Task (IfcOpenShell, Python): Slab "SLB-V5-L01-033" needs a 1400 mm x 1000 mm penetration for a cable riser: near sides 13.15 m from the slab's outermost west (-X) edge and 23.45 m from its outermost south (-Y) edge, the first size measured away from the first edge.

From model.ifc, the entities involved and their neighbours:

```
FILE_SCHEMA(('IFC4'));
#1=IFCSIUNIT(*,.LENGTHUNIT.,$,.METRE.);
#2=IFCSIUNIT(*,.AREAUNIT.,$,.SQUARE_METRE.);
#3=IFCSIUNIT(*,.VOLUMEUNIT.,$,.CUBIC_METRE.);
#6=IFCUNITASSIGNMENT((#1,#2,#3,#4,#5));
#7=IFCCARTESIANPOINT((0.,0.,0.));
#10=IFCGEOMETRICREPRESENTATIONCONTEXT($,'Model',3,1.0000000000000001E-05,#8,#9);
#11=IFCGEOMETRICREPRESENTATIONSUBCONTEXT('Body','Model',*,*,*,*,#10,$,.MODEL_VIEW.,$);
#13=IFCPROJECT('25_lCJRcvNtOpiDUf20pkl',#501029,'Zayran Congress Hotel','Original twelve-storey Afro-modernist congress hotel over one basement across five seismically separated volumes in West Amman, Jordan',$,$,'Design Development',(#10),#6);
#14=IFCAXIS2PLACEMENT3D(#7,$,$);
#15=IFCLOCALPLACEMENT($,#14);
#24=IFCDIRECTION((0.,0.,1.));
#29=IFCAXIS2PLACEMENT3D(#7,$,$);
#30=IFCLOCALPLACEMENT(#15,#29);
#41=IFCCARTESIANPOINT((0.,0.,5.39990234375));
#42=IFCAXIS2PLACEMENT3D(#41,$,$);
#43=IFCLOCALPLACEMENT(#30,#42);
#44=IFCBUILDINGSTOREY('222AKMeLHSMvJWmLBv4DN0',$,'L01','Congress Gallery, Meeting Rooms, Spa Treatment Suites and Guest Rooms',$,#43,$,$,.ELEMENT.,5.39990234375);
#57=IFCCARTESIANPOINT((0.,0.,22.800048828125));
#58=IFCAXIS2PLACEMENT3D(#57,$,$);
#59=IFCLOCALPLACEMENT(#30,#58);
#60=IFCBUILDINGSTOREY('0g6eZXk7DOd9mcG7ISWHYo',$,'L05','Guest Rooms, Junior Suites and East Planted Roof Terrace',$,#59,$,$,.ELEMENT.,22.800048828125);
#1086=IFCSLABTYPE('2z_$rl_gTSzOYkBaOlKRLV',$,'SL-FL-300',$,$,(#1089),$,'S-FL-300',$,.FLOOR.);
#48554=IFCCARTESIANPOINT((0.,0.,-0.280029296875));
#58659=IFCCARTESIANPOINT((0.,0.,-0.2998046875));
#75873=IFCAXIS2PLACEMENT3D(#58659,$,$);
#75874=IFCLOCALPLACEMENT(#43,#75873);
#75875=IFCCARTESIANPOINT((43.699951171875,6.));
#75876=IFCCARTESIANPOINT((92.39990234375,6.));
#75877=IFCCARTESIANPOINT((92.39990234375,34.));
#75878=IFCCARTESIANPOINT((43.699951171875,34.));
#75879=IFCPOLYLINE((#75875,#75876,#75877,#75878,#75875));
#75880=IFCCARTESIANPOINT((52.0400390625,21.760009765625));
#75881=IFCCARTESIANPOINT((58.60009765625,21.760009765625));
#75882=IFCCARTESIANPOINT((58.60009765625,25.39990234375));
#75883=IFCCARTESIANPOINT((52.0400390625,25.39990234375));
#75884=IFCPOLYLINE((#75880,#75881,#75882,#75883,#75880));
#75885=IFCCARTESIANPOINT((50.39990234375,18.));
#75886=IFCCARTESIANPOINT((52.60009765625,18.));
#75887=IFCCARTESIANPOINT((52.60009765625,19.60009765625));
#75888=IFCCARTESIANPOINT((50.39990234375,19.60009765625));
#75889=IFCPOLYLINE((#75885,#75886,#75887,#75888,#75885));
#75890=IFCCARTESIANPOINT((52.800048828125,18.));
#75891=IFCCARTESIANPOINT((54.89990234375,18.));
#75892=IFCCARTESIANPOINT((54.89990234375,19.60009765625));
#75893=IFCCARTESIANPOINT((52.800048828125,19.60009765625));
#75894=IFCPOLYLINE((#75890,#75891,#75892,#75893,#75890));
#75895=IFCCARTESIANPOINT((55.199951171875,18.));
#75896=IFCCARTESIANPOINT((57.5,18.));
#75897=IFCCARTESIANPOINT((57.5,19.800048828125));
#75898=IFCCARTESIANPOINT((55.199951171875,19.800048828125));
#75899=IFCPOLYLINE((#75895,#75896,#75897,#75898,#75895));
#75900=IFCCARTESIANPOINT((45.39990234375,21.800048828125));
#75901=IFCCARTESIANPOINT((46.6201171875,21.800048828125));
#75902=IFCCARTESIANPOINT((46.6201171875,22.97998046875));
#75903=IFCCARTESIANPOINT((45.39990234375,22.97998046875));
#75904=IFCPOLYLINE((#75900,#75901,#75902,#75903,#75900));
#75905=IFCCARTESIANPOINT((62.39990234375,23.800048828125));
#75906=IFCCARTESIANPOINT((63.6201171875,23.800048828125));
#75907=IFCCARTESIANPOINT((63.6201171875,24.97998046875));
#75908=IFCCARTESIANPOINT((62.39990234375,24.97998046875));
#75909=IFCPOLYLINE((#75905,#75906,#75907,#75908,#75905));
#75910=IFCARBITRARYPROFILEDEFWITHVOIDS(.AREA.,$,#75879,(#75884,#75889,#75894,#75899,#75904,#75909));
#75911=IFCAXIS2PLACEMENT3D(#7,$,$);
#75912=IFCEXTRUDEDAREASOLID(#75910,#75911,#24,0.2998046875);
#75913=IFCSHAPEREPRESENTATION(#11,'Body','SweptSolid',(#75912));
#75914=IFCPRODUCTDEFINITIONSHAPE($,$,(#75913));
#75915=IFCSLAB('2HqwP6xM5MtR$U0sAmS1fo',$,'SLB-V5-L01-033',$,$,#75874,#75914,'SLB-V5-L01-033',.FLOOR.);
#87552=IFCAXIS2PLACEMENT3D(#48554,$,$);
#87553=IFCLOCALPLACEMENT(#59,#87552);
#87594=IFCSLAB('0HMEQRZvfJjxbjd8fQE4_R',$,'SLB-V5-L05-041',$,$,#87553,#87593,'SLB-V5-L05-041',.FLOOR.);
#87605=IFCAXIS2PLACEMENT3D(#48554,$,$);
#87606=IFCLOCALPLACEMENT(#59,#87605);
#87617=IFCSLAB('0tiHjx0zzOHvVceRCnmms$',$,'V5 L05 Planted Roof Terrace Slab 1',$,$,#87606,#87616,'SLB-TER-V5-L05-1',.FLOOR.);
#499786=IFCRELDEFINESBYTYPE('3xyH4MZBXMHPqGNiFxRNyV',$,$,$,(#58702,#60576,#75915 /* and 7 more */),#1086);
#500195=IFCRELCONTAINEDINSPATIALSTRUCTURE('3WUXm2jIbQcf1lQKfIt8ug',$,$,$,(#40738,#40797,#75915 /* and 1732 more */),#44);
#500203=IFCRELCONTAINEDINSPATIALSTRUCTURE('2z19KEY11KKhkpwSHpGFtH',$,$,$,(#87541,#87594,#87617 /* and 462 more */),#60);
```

```python
import numpy as np
import ifcopenshell
import ifcopenshell.api.feature
import ifcopenshell.api.geometry
import ifcopenshell.api.root
import ifcopenshell.geom
import ifcopenshell.util.placement
import ifcopenshell.util.representation
import ifcopenshell.util.shape
import ifcopenshell.util.unit

model = ifcopenshell.open("model.ifc")
unit_scale = ifcopenshell.util.unit.calculate_unit_scale(model)
settings = ifcopenshell.geom.settings()


def volume(element):
    """Net volume in cubic metres, openings subtracted."""
    shape = ifcopenshell.geom.create_shape(settings, element)
    return ifcopenshell.util.shape.get_volume(shape.geometry)


slab = model.by_id(75915)
before = volume(slab)

# Extent in the slab's own axes, in metres. The edges named are its -X and -Y sides.
slab_shape = ifcopenshell.geom.create_shape(settings, slab)
vertices = ifcopenshell.util.shape.get_vertices(slab_shape.geometry)
x_min, y_min, bottom = vertices.min(axis=0)
top = vertices[:, 2].max()

opening = ifcopenshell.api.root.create_entity(model, ifc_class="IfcOpeningElement", name="Cable riser opening", predefined_type="OPENING")
context = ifcopenshell.util.representation.get_context(model, "Model", "Body", "MODEL_VIEW")
width, depth = 1.4, 1
outline = [(0.0, 0.0), (width, 0.0), (width, depth), (0.0, depth), (0.0, 0.0)]
# Overshoot both faces by 50 mm so the cut is clean.
shape = ifcopenshell.api.geometry.add_slab_representation(
    model, context=context, depth=top - bottom + 0.1, polyline=outline
)
ifcopenshell.api.geometry.assign_representation(model, product=opening, representation=shape)

matrix = ifcopenshell.util.placement.get_local_placement(slab.ObjectPlacement)
matrix[:, 3] = matrix @ np.append(np.array([x_min + 13.15, y_min + 23.45, bottom - 0.05]) / unit_scale, 1.0)
ifcopenshell.api.geometry.edit_object_placement(model, product=opening, matrix=matrix, is_si=False)
ifcopenshell.api.feature.add_feature(model, feature=opening, element=slab)

after = volume(slab)

print(f"slab volume {before:.3f} -> {after:.3f} m3")

model.write("model_updated.ifc")
```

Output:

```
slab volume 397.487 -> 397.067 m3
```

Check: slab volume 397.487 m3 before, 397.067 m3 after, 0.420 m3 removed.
